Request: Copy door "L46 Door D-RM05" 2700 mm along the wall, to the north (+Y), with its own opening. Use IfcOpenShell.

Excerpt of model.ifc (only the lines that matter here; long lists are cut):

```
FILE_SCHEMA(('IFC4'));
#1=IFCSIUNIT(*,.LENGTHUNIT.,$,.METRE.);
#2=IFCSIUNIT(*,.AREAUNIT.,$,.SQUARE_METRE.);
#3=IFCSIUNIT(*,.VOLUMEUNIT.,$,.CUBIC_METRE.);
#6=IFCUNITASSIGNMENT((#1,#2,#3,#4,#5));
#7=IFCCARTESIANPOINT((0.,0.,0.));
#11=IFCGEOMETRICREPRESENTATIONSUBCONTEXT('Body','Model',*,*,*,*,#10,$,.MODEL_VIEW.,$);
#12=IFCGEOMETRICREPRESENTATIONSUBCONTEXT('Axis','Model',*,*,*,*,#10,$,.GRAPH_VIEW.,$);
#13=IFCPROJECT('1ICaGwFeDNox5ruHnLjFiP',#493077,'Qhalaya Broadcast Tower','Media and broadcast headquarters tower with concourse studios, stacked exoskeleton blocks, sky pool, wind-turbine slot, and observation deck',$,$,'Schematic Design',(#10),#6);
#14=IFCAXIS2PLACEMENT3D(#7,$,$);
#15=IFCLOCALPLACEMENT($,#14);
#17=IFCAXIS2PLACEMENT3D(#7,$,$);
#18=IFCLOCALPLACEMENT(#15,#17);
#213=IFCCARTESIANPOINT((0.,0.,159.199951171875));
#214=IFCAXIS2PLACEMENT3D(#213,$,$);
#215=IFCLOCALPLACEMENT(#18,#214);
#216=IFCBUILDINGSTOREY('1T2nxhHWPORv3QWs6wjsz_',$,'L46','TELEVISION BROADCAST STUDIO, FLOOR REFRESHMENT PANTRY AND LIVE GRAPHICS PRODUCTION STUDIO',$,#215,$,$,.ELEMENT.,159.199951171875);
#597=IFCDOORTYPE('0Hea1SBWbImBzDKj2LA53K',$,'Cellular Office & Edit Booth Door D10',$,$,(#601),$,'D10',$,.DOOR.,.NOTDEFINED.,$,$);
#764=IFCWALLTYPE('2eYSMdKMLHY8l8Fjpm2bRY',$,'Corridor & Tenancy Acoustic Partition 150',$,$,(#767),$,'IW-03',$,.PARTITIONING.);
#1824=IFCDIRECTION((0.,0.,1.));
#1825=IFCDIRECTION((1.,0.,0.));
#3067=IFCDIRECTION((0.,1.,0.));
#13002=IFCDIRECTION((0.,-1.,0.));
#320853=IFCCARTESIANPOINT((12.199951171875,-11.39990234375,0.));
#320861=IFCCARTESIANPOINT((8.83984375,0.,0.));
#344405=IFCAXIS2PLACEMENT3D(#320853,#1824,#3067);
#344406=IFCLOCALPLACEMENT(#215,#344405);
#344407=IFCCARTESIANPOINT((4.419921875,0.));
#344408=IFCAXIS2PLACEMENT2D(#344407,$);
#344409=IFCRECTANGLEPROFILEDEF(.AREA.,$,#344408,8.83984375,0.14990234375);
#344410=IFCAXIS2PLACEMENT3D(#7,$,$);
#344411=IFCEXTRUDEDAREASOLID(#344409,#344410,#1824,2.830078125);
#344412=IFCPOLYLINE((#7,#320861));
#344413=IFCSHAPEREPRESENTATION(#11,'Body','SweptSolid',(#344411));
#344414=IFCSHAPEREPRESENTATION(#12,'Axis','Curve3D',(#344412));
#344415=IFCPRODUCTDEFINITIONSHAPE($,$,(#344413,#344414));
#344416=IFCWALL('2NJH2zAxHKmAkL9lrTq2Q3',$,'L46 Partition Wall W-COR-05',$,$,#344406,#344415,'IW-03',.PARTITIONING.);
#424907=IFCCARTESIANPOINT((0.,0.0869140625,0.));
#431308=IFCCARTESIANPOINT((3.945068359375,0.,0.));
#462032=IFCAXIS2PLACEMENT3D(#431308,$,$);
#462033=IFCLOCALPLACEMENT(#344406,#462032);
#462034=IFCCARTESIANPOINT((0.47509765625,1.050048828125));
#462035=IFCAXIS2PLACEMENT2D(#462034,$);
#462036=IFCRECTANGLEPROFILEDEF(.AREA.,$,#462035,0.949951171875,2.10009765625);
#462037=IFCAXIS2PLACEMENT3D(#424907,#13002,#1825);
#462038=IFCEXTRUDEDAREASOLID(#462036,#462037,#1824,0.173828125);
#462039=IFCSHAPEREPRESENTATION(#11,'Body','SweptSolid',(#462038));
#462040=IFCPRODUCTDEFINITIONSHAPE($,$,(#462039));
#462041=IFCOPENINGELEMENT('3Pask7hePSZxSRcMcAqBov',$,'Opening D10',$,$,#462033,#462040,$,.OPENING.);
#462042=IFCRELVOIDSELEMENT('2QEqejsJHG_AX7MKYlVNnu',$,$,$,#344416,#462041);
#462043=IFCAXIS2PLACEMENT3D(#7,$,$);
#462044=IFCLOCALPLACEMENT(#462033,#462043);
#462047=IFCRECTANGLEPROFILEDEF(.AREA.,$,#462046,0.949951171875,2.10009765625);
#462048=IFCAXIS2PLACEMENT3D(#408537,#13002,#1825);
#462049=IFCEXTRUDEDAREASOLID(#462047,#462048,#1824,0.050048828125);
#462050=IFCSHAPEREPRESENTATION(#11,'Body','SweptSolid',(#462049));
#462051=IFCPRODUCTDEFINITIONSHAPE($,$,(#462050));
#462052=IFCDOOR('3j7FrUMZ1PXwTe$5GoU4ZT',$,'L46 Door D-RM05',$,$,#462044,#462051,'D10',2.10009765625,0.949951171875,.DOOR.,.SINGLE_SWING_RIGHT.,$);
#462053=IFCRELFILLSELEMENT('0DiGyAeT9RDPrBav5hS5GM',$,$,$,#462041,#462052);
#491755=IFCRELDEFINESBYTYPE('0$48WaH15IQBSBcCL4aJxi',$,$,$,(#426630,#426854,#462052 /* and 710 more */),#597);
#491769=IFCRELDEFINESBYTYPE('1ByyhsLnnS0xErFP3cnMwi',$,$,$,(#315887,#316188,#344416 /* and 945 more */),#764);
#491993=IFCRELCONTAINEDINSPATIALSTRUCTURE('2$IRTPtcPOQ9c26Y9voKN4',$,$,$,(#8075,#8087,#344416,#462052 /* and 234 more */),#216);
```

```python
import ifcopenshell
import ifcopenshell.api.feature
import ifcopenshell.api.geometry
import ifcopenshell.api.root
import ifcopenshell.geom
import ifcopenshell.util.element
import ifcopenshell.util.placement
import ifcopenshell.util.shape
import ifcopenshell.util.unit

model = ifcopenshell.open("model.ifc")
unit_scale = ifcopenshell.util.unit.calculate_unit_scale(model)
settings = ifcopenshell.geom.settings()


def volume(element):
    """Net volume in cubic metres, openings subtracted."""
    shape = ifcopenshell.geom.create_shape(settings, element)
    return ifcopenshell.util.shape.get_volume(shape.geometry)


door = model.by_guid("3j7FrUMZ1PXwTe$5GoU4ZT")
opening = door.FillsVoids[0].RelatingOpeningElement
wall = opening.VoidsElements[0].RelatingBuildingElement
before = volume(wall)
shift = ifcopenshell.util.placement.get_local_placement(wall.ObjectPlacement)[:3, 0] * 2.7 / unit_scale

# copy_class copies the void relationship, type, container and properties, but no geometry.
new_opening = ifcopenshell.api.root.copy_class(model, product=opening)
new_opening.Representation = ifcopenshell.util.element.copy_deep(
    model, opening.Representation, exclude=["IfcGeometricRepresentationContext", "IfcRepresentationMap"]
)
new_door = ifcopenshell.api.root.copy_class(model, product=door)
new_door.Representation = ifcopenshell.util.element.copy_deep(
    model, door.Representation, exclude=["IfcGeometricRepresentationContext", "IfcRepresentationMap"]
)
new_door.Tag = None
ifcopenshell.api.feature.add_filling(model, opening=new_opening, element=new_door)

for old, new in ((opening, new_opening), (door, new_door)):
    matrix = ifcopenshell.util.placement.get_local_placement(old.ObjectPlacement)
    matrix[:3, 3] += shift
    ifcopenshell.api.geometry.edit_object_placement(model, product=new, matrix=matrix, is_si=False)

after = volume(wall)

print(f"wall volume {before:.3f} -> {after:.3f} m3")

model.write("model_rev.ifc")
```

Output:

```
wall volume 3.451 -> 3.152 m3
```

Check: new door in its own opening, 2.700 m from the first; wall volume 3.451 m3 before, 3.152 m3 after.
